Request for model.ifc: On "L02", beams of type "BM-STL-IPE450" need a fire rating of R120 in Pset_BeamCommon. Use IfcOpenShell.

First a look at what the model holds.

```python
import ifcopenshell
import ifcopenshell.util.element

model = ifcopenshell.open("model.ifc")
print(model.schema)
storey = next(s for s in model.by_type("IfcBuildingStorey") if s.Name == "L02")
beams = [e for e in ifcopenshell.util.element.get_decomposition(storey) if e.is_a("IfcBeam")]
seen = {}
for e in beams:
    element_type = ifcopenshell.util.element.get_type(e)
    key = (element_type.Name if element_type != e and element_type else None, ifcopenshell.util.element.get_pset(e, "Pset_BeamCommon", "FireRating"))
    seen[key] = seen.get(key, 0) + 1
for (name, value), count in sorted(seen.items(), key=str):
    print(count, "x", name, "|", value)
```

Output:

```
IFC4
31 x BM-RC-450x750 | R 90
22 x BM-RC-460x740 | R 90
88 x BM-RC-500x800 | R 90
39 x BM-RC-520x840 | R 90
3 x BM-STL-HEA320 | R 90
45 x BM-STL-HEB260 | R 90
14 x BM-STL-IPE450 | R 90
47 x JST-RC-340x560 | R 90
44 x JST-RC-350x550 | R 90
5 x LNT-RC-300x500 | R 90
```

```python
import ifcopenshell
import ifcopenshell.api.pset
import ifcopenshell.util.element

model = ifcopenshell.open("model.ifc")

storey = next(s for s in model.by_type("IfcBuildingStorey") if s.Name == "L02")
beams = [e for e in ifcopenshell.util.element.get_decomposition(storey) if e.is_a("IfcBeam")]

count = 0
for e in beams:
    element_type = ifcopenshell.util.element.get_type(e)
    if element_type in (None, e) or element_type.Name != "BM-STL-IPE450":
        continue
    # add_pset returns the element's existing set when there is one.
    pset = ifcopenshell.api.pset.add_pset(model, product=e, name="Pset_BeamCommon")
    ifcopenshell.api.pset.edit_pset(model, pset=pset, properties={"FireRating": "R120"})
    count += 1

print(count, "beams updated")

model.write("model_v2.ifc")
```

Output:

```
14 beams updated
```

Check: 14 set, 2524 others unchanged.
